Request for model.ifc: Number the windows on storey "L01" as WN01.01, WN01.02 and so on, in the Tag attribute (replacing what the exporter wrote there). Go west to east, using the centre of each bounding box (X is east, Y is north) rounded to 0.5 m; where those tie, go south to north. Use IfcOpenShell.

First a look at what the model holds.

```python
import ifcopenshell
import ifcopenshell.util.element
import ifcopenshell.util.placement

model = ifcopenshell.open("model.ifc")
print(model.schema)
storey = next(s for s in model.by_type("IfcBuildingStorey") if s.Name == "L01")
windows = [e for e in ifcopenshell.util.element.get_decomposition(storey) if e.is_a("IfcWindow")]
for e in sorted(windows, key=lambda e: e.id()):
    origin = ifcopenshell.util.placement.get_local_placement(e.ObjectPlacement)[:3, 3]
    print(e.id(), e.Tag, e.Name, origin.round(2) + 0.0, sep=" | ")
```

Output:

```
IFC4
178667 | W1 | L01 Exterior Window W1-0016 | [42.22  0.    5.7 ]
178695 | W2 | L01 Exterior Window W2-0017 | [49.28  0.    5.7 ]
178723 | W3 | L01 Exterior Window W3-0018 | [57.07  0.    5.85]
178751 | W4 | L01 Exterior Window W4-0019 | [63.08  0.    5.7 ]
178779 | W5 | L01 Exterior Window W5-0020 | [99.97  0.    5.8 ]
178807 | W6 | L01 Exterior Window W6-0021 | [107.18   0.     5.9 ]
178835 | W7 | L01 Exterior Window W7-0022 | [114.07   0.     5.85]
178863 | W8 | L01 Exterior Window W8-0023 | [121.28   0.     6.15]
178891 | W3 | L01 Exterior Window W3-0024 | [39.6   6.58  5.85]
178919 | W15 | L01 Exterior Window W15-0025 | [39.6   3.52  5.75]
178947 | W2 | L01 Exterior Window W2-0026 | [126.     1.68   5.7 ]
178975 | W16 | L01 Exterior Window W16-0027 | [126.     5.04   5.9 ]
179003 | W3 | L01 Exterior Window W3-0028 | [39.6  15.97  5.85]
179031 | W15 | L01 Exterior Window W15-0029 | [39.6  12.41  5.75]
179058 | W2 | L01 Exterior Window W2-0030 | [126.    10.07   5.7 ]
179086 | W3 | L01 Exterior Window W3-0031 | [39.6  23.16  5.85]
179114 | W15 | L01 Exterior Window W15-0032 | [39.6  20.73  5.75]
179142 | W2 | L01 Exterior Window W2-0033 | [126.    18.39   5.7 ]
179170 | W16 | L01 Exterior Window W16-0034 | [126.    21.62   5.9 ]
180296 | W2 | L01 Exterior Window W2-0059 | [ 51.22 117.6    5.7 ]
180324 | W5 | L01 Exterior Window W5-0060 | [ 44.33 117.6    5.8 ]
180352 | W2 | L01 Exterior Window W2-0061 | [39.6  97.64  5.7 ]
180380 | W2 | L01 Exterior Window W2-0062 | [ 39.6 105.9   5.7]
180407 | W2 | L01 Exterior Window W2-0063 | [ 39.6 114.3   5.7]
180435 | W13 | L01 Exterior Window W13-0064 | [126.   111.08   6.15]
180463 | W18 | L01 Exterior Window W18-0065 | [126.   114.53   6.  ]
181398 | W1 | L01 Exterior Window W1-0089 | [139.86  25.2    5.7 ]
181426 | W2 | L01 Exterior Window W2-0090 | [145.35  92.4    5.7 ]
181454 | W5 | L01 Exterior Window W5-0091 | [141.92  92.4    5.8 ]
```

```python
import ifcopenshell
import ifcopenshell.geom
import ifcopenshell.util.element
import ifcopenshell.util.shape

model = ifcopenshell.open("model.ifc")
settings = ifcopenshell.geom.settings()
settings.set("use-world-coords", True)


def centre(element):
    shape = ifcopenshell.geom.create_shape(settings, element)
    return ifcopenshell.util.shape.get_bbox_centroid(shape.geometry)


storey = next(s for s in model.by_type("IfcBuildingStorey") if s.Name == "L01")
windows = [e for e in ifcopenshell.util.element.get_decomposition(storey) if e.is_a("IfcWindow")]

# Insertion points can sit at a corner or the storey origin, so sort by the geometry (in metres).
centres = {e: centre(e) for e in windows}
windows.sort(key=lambda e: (round(centres[e][0] / 0.5), centres[e][1]))

for i, e in enumerate(windows, start=1):
    number = f"WN01.{i:02d}"
    e.Tag = number
    print(e.id(), number)

model.write("model_rev.ifc")
```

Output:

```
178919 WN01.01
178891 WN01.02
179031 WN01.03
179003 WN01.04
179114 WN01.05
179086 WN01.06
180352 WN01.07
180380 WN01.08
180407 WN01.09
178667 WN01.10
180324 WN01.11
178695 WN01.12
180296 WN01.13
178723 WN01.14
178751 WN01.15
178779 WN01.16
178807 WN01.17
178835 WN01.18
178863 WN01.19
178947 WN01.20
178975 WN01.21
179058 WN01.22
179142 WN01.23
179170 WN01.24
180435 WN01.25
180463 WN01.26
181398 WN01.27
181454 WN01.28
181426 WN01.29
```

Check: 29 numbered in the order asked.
